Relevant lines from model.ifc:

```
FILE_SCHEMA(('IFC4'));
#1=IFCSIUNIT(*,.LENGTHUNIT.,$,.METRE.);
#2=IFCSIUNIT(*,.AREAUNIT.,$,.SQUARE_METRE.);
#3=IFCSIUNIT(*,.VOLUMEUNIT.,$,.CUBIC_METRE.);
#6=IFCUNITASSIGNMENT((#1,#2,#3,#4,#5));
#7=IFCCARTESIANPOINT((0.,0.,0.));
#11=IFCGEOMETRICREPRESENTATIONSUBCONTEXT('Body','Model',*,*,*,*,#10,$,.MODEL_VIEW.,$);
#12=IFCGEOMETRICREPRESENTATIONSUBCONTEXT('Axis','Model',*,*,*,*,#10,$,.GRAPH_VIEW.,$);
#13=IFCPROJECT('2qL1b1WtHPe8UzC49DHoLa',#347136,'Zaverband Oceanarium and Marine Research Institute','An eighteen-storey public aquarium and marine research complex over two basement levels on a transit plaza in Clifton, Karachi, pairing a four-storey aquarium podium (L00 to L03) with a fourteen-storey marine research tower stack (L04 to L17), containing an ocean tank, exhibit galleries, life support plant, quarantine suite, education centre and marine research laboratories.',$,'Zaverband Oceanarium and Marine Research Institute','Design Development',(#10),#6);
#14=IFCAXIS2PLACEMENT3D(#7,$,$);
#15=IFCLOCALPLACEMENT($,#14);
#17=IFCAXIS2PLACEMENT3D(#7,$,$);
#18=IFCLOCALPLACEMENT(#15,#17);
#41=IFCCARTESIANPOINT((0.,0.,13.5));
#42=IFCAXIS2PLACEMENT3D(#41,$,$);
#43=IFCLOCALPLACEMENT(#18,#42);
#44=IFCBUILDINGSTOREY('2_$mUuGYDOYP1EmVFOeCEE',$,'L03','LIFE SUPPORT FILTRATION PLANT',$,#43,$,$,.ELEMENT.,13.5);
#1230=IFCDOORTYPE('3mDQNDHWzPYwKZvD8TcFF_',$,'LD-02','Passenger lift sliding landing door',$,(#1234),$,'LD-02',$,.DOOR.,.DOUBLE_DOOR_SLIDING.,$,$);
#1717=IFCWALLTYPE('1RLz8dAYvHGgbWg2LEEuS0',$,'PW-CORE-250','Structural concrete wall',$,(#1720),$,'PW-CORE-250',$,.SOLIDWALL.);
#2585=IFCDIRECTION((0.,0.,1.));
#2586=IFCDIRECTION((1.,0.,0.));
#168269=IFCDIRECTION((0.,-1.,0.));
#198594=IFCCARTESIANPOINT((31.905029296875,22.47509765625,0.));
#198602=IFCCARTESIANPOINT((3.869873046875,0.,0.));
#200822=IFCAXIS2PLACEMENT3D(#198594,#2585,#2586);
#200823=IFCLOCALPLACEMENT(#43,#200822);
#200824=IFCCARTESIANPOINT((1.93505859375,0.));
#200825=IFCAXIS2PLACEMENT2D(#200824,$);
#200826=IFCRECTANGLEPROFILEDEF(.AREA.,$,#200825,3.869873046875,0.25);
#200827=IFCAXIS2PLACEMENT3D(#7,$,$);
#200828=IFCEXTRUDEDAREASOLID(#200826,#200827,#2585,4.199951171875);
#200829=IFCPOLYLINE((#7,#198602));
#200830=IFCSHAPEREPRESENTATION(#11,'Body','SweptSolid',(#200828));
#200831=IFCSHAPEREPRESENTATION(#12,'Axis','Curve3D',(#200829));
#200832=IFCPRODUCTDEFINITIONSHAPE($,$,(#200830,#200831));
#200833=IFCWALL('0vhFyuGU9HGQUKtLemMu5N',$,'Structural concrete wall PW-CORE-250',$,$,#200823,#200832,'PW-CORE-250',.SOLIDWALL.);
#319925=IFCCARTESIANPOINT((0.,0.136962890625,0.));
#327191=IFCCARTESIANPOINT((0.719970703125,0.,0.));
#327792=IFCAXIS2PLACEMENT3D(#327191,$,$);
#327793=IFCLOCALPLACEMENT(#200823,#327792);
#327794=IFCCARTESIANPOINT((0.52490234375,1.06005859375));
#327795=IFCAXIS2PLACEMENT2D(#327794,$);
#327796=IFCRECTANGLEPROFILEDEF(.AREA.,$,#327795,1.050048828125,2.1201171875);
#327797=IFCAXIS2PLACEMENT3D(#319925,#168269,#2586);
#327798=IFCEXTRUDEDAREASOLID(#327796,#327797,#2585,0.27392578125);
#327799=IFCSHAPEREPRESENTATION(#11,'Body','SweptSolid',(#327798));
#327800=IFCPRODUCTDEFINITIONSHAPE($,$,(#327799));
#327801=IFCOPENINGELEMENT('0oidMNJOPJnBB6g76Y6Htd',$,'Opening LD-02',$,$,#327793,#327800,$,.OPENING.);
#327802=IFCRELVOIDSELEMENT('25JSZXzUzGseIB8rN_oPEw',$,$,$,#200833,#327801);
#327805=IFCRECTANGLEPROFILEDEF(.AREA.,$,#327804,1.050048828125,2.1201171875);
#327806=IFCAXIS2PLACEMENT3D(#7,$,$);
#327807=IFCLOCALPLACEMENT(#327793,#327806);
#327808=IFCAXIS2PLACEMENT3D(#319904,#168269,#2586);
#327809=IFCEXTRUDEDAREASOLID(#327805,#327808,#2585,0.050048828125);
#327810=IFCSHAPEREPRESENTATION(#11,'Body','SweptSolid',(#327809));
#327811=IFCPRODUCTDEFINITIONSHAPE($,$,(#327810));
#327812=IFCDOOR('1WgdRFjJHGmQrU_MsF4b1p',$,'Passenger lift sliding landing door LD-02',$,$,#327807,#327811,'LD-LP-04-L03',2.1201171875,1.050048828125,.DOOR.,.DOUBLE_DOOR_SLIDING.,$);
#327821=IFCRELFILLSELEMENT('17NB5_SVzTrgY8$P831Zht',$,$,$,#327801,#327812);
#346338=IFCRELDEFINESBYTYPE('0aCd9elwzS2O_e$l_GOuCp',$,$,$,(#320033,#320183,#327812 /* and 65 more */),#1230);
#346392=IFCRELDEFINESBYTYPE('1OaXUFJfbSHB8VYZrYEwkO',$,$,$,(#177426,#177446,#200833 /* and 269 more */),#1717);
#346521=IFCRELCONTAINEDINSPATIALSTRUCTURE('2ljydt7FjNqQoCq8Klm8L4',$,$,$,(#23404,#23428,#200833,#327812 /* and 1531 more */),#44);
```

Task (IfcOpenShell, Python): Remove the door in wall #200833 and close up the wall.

```python
import ifcopenshell
import ifcopenshell.api.feature
import ifcopenshell.api.root
import ifcopenshell.geom
import ifcopenshell.util.shape

model = ifcopenshell.open("model.ifc")
settings = ifcopenshell.geom.settings()


def volume(element):
    """Net volume in cubic metres, openings subtracted."""
    shape = ifcopenshell.geom.create_shape(settings, element)
    return ifcopenshell.util.shape.get_volume(shape.geometry)


door = model.by_guid("1WgdRFjJHGmQrU_MsF4b1p")
opening = door.FillsVoids[0].RelatingOpeningElement
wall = opening.VoidsElements[0].RelatingBuildingElement
before = volume(wall)

ifcopenshell.api.root.remove_product(model, product=door)
ifcopenshell.api.feature.remove_feature(model, feature=opening)

after = volume(wall)

print(f"wall volume {before:.3f} -> {after:.3f} m3")

model.write("model_v2.ifc")
```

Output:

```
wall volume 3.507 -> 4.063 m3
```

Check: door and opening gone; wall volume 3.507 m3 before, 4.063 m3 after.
